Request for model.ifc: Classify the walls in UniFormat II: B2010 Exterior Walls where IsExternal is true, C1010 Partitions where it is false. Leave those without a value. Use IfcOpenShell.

First a look at what the model holds.

```python
import ifcopenshell
import ifcopenshell.util.element

model = ifcopenshell.open("model.ifc")
print(model.schema)
print("classifications:", [c.Name for c in model.by_type("IfcClassification")])
values = [ifcopenshell.util.element.get_pset(e, "Pset_WallCommon", "IsExternal") for e in model.by_type("IfcWall")]
for value in (True, False, None):
    print("IsExternal", value, values.count(value))
```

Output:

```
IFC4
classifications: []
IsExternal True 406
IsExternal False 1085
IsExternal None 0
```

```python
import ifcopenshell
import ifcopenshell.api.classification
import ifcopenshell.util.element

model = ifcopenshell.open("model.ifc")

system = ifcopenshell.api.classification.add_classification(model, classification="UniFormat II")

walls = model.by_type("IfcWall")
external = {e: ifcopenshell.util.element.get_pset(e, "Pset_WallCommon", "IsExternal") for e in walls}
for flag, code, name in ((True, "B2010", "Exterior Walls"), (False, "C1010", "Partitions")):
    products = [e for e in walls if external[e] is flag]
    ifcopenshell.api.classification.add_reference(
        model, products=products, classification=system, identification=code, name=name
    )
    print(code, len(products))

model.write("model-out.ifc")
```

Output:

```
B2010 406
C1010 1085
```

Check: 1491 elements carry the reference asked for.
